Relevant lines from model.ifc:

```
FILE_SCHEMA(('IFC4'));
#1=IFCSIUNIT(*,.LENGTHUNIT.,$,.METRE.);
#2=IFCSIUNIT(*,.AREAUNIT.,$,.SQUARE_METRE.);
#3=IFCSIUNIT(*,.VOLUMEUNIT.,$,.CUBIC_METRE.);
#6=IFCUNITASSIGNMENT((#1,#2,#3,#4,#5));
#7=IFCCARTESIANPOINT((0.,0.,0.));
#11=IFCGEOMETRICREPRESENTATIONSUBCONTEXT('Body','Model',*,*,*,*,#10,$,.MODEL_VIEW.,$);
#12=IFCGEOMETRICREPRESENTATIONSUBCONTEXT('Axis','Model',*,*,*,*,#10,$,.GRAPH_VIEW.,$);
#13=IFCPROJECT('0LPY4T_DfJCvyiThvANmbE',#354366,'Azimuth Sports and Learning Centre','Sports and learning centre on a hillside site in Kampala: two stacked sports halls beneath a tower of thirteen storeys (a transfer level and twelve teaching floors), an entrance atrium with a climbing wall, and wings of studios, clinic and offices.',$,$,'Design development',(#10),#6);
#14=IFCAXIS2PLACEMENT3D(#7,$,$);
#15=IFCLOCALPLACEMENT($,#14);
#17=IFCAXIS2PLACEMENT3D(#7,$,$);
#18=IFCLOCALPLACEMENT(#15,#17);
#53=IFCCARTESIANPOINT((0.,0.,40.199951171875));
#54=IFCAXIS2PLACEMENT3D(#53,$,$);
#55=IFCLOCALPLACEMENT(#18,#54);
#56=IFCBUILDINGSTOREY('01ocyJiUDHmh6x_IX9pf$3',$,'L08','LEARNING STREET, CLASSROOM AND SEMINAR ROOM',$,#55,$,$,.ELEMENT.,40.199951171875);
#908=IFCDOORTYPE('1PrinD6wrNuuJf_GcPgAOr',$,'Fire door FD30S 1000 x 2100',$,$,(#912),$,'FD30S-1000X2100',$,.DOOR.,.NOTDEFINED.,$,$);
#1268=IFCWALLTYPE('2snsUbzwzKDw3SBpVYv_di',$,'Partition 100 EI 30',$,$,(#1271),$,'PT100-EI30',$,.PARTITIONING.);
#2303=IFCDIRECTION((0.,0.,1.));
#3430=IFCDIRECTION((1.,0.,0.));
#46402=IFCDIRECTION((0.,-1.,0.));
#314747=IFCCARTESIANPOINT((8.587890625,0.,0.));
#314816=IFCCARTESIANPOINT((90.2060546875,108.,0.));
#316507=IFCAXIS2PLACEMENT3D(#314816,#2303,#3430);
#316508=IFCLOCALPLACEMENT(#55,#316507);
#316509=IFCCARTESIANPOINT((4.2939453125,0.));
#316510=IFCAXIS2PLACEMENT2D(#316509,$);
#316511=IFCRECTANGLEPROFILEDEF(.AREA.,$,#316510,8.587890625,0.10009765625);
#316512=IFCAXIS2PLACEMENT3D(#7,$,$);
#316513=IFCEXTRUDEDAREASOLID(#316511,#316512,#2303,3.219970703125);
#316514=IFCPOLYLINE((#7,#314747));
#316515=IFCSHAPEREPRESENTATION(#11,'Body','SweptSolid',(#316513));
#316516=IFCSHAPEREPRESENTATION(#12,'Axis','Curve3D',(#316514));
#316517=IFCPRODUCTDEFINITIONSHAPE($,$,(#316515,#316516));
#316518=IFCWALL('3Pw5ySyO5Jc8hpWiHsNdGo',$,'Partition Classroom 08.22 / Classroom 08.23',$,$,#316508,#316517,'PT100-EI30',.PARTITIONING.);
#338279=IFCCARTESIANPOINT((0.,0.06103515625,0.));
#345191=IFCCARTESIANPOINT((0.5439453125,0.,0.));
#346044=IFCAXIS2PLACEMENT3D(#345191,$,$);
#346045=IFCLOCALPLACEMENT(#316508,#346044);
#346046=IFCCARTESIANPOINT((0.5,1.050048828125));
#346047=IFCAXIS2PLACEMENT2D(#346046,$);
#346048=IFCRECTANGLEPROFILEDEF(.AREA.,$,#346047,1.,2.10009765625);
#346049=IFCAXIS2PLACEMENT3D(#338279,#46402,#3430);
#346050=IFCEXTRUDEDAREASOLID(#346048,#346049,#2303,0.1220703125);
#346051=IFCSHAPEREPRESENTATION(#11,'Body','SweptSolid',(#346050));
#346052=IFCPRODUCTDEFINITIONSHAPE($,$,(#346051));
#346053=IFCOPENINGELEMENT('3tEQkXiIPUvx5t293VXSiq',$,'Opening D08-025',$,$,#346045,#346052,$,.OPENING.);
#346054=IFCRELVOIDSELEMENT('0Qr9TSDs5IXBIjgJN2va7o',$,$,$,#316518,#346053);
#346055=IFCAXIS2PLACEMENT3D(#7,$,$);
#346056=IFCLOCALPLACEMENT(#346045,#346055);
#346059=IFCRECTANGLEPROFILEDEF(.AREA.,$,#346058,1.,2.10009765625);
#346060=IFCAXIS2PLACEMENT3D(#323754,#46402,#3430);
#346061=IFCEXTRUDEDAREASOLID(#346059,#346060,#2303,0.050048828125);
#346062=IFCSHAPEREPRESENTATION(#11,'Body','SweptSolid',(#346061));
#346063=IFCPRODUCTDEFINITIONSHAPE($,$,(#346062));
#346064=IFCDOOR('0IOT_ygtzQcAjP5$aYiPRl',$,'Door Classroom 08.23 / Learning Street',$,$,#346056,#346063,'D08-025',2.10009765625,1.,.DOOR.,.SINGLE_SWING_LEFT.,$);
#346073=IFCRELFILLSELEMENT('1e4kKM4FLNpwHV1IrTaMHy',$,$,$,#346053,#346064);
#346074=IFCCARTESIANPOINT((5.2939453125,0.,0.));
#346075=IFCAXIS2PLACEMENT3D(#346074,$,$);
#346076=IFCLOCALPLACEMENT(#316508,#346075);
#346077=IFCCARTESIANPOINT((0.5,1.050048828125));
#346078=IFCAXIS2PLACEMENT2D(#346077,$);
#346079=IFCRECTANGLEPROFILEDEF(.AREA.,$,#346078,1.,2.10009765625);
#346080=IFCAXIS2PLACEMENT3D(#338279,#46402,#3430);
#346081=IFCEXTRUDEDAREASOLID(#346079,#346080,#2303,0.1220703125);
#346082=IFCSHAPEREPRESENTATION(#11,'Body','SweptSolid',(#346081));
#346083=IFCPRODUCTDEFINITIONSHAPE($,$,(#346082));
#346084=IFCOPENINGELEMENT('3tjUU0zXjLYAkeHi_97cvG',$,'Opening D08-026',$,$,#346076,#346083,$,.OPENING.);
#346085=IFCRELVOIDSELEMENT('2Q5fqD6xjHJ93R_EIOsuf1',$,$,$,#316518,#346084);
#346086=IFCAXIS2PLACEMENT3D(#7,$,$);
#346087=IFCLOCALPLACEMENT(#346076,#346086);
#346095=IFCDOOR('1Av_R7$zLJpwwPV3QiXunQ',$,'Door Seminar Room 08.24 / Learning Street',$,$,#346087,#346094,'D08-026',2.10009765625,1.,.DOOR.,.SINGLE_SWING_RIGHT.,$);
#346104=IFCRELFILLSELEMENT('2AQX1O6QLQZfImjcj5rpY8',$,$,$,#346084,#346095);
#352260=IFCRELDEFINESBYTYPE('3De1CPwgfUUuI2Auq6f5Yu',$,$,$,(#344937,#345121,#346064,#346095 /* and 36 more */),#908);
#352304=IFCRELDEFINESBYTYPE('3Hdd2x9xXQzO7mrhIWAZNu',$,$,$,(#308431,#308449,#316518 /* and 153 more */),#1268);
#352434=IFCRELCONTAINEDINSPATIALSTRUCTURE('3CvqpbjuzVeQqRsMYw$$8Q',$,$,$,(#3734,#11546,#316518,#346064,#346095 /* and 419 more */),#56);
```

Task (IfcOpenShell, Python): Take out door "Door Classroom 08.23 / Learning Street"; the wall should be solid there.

```python
import ifcopenshell
import ifcopenshell.api.feature
import ifcopenshell.api.root
import ifcopenshell.geom
import ifcopenshell.util.shape

model = ifcopenshell.open("model.ifc")
settings = ifcopenshell.geom.settings()


def volume(element):
    """Net volume in cubic metres, openings subtracted."""
    shape = ifcopenshell.geom.create_shape(settings, element)
    return ifcopenshell.util.shape.get_volume(shape.geometry)


door = model.by_guid("0IOT_ygtzQcAjP5$aYiPRl")
opening = door.FillsVoids[0].RelatingOpeningElement
wall = opening.VoidsElements[0].RelatingBuildingElement
before = volume(wall)

ifcopenshell.api.root.remove_product(model, product=door)
ifcopenshell.api.feature.remove_feature(model, feature=opening)

after = volume(wall)

print(f"wall volume {before:.3f} -> {after:.3f} m3")

model.write("model_edited.ifc")
```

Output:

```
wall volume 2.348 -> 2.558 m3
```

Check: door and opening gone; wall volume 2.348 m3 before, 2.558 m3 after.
